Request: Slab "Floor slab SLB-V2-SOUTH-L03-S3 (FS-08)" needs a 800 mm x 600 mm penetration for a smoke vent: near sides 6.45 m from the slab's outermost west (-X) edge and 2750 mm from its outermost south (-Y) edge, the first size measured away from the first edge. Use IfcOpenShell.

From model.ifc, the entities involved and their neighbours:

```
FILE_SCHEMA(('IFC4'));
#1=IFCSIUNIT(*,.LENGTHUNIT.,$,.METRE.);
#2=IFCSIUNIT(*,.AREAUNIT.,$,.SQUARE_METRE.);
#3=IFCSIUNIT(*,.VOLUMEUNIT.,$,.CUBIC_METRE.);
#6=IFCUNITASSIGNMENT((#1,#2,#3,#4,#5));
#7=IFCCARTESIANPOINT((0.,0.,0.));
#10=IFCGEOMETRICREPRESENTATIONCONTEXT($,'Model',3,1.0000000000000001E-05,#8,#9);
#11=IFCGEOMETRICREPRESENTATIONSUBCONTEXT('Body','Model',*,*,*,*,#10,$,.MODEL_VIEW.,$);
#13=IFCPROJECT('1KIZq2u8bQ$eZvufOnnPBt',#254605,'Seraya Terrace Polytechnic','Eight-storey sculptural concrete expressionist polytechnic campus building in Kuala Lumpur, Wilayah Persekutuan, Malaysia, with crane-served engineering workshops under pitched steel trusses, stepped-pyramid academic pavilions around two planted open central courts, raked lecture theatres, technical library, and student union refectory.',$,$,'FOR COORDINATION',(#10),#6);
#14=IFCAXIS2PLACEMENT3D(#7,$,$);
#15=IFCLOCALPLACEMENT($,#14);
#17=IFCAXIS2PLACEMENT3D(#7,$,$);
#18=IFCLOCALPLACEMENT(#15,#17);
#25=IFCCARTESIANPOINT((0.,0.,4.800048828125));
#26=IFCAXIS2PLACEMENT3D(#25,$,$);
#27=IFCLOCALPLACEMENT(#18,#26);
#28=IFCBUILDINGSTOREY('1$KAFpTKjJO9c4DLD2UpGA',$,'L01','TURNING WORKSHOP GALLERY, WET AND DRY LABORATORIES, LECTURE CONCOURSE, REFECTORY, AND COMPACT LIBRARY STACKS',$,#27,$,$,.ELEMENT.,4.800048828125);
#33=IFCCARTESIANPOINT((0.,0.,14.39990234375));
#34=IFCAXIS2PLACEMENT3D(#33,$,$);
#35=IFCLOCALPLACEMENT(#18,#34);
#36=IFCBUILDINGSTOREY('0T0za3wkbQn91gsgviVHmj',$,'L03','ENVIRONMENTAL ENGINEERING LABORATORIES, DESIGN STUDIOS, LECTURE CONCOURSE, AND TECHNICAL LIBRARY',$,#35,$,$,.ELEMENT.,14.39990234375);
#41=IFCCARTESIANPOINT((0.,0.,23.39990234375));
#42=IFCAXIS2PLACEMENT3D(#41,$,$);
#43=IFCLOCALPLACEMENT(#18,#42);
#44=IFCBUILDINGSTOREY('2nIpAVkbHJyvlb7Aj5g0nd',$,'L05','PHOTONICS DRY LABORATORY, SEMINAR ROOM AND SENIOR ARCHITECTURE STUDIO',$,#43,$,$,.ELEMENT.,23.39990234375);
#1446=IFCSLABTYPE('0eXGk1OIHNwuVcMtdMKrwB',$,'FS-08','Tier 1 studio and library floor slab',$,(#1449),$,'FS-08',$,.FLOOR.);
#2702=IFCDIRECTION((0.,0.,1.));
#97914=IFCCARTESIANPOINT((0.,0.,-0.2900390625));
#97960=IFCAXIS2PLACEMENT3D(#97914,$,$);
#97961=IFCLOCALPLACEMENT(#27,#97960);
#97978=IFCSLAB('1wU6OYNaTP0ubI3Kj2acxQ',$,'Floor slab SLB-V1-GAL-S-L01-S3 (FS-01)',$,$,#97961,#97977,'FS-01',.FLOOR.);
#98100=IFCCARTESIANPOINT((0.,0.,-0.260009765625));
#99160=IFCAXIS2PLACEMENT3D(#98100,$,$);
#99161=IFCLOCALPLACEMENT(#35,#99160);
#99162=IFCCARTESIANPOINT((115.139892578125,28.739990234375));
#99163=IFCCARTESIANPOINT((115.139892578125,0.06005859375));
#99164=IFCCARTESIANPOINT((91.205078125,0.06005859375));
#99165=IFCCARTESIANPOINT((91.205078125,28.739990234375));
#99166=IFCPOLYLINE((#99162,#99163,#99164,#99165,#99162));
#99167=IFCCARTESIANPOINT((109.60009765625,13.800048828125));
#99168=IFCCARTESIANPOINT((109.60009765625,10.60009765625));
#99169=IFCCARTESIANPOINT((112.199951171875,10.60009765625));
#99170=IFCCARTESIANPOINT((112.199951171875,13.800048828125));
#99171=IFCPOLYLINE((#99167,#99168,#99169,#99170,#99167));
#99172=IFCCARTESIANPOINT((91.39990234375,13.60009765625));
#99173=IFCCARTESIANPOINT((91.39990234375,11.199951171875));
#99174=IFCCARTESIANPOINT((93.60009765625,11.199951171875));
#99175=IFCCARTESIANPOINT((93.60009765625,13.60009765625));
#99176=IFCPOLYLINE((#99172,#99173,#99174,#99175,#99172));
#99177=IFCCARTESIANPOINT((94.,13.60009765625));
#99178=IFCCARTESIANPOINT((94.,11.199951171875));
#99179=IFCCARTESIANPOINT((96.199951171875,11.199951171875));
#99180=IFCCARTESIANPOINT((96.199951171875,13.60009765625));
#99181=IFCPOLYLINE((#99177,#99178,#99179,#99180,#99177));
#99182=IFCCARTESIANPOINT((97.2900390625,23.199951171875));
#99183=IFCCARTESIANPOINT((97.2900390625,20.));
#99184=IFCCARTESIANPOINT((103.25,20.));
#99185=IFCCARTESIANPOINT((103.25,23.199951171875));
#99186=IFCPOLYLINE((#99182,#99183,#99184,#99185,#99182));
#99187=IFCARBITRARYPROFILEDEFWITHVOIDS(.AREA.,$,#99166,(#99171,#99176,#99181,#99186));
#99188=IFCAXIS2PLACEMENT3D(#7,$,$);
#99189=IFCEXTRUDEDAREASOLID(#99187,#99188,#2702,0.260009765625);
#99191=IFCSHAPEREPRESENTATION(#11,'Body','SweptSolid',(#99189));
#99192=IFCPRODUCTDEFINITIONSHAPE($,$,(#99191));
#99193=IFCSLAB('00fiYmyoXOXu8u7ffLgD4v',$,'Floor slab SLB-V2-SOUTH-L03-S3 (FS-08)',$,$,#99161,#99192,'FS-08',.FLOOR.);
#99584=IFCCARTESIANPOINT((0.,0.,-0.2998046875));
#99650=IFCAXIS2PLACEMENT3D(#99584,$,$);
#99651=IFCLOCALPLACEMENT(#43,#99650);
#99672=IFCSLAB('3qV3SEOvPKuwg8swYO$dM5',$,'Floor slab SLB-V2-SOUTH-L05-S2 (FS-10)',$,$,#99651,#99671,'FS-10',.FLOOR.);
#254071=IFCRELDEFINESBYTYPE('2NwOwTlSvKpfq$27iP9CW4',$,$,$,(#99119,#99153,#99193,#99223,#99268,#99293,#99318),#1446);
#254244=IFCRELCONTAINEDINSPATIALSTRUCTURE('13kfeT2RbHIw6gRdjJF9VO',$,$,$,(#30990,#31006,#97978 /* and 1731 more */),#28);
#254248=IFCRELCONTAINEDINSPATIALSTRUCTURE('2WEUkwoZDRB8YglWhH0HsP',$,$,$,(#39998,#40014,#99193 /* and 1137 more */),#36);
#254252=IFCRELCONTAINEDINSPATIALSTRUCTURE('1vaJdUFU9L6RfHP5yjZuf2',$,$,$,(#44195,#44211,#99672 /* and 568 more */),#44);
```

```python
import numpy as np
import ifcopenshell
import ifcopenshell.api.feature
import ifcopenshell.api.geometry
import ifcopenshell.api.root
import ifcopenshell.geom
import ifcopenshell.util.placement
import ifcopenshell.util.representation
import ifcopenshell.util.shape
import ifcopenshell.util.unit

model = ifcopenshell.open("model.ifc")
unit_scale = ifcopenshell.util.unit.calculate_unit_scale(model)
settings = ifcopenshell.geom.settings()


def volume(element):
    """Net volume in cubic metres, openings subtracted."""
    shape = ifcopenshell.geom.create_shape(settings, element)
    return ifcopenshell.util.shape.get_volume(shape.geometry)


slab = model.by_guid("00fiYmyoXOXu8u7ffLgD4v")
before = volume(slab)

# Extent in the slab's own axes, in metres. The edges named are its -X and -Y sides.
slab_shape = ifcopenshell.geom.create_shape(settings, slab)
vertices = ifcopenshell.util.shape.get_vertices(slab_shape.geometry)
x_min, y_min, bottom = vertices.min(axis=0)
top = vertices[:, 2].max()

opening = ifcopenshell.api.root.create_entity(model, ifc_class="IfcOpeningElement", name="Smoke vent opening", predefined_type="OPENING")
context = ifcopenshell.util.representation.get_context(model, "Model", "Body", "MODEL_VIEW")
width, depth = 0.8, 0.6
outline = [(0.0, 0.0), (width, 0.0), (width, depth), (0.0, depth), (0.0, 0.0)]
# Overshoot both faces by 50 mm so the cut is clean.
shape = ifcopenshell.api.geometry.add_slab_representation(
    model, context=context, depth=top - bottom + 0.1, polyline=outline
)
ifcopenshell.api.geometry.assign_representation(model, product=opening, representation=shape)

matrix = ifcopenshell.util.placement.get_local_placement(slab.ObjectPlacement)
matrix[:, 3] = matrix @ np.append(np.array([x_min + 6.45, y_min + 2.75, bottom - 0.05]) / unit_scale, 1.0)
ifcopenshell.api.geometry.edit_object_placement(model, product=opening, matrix=matrix, is_si=False)
ifcopenshell.api.feature.add_feature(model, feature=opening, element=slab)

after = volume(slab)

print(f"slab volume {before:.3f} -> {after:.3f} m3")

model.write("model-out.ifc")
```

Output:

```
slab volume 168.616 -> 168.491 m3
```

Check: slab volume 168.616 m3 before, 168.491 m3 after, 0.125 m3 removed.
